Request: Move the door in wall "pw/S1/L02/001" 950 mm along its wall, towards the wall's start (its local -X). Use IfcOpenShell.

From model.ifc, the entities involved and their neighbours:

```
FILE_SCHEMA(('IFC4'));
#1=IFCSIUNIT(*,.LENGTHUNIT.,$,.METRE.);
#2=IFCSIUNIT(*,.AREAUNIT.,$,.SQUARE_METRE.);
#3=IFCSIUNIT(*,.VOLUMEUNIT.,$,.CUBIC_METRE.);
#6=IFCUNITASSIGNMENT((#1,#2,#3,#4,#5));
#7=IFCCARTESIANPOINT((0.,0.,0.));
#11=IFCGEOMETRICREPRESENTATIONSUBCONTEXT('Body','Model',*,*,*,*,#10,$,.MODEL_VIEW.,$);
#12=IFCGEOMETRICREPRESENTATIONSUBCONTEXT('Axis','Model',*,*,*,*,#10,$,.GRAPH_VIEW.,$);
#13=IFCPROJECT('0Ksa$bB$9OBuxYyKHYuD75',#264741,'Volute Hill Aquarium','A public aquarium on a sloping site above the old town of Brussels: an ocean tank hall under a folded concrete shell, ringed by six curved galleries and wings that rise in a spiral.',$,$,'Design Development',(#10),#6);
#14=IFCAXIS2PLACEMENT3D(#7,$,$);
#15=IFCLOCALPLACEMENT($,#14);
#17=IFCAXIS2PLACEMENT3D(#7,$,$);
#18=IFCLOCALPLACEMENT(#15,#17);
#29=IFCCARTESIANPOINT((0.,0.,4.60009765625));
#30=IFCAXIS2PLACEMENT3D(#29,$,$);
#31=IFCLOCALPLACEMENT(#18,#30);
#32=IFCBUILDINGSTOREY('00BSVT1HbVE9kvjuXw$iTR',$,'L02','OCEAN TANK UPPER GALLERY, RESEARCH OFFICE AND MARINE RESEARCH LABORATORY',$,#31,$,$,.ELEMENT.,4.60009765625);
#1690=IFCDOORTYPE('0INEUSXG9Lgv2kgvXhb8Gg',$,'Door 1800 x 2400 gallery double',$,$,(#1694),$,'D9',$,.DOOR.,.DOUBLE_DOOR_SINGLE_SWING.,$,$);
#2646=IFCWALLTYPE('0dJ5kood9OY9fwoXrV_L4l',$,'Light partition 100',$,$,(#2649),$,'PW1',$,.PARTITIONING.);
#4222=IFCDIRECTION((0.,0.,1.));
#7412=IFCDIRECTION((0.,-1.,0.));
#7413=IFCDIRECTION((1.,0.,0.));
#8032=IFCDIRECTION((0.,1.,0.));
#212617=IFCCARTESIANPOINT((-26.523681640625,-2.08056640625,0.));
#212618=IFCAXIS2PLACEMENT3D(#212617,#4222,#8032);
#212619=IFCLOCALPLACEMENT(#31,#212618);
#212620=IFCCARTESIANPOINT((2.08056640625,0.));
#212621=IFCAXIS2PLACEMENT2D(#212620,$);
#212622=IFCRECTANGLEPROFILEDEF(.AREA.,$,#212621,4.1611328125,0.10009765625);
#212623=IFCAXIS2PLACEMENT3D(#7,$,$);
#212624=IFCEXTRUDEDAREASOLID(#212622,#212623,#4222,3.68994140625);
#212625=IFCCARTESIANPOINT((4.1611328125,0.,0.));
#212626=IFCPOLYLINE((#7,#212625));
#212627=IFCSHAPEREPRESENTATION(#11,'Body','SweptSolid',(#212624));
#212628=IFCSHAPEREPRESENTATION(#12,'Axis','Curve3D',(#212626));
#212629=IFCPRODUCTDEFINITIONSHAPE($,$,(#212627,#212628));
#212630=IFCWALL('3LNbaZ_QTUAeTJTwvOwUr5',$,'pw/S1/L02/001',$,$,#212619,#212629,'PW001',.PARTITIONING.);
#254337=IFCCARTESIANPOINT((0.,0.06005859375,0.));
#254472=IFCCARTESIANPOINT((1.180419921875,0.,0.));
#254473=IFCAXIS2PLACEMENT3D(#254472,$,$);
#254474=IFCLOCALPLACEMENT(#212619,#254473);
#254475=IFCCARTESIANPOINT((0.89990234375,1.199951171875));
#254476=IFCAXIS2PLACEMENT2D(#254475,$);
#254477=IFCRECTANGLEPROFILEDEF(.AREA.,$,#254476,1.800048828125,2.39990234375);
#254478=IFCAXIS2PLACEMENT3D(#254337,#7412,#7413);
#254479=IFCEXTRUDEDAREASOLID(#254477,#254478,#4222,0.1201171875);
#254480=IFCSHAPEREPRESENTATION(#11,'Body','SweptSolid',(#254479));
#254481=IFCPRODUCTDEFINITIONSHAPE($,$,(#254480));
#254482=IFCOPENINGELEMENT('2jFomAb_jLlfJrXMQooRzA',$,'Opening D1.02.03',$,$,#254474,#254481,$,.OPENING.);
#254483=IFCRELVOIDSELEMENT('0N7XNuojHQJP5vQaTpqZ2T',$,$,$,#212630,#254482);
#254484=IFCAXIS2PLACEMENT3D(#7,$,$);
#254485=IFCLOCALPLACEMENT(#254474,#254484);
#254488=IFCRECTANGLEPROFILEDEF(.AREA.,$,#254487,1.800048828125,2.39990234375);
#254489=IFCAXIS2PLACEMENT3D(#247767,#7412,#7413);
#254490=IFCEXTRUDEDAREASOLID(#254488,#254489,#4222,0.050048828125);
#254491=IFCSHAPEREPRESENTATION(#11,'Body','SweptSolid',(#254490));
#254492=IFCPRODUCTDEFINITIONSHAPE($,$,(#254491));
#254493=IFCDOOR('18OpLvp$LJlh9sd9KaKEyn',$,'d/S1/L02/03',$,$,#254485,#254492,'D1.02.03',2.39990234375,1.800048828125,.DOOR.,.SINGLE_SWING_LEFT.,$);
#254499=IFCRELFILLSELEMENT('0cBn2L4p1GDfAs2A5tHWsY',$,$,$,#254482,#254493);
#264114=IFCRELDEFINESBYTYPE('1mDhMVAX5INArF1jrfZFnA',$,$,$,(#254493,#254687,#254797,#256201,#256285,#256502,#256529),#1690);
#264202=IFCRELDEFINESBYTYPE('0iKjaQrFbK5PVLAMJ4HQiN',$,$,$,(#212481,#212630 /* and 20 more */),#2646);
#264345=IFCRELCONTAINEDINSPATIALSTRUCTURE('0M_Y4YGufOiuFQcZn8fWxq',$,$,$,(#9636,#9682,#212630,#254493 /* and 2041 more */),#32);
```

```python
import ifcopenshell
import ifcopenshell.api.geometry
import ifcopenshell.util.placement
import ifcopenshell.util.unit

model = ifcopenshell.open("model.ifc")
unit_scale = ifcopenshell.util.unit.calculate_unit_scale(model)

door = model.by_id(254493)
opening = door.FillsVoids[0].RelatingOpeningElement
wall = opening.VoidsElements[0].RelatingBuildingElement

wall_matrix = ifcopenshell.util.placement.get_local_placement(wall.ObjectPlacement)
shift = wall_matrix[:3, 0] * -0.95 / unit_scale
before = ifcopenshell.util.placement.get_local_placement(door.ObjectPlacement)[:3, 3].copy()

# The door is placed relative to its opening, so it follows when the opening moves.
matrix = ifcopenshell.util.placement.get_local_placement(opening.ObjectPlacement)
matrix[:3, 3] += shift
ifcopenshell.api.geometry.edit_object_placement(
    model, product=opening, matrix=matrix, is_si=False, should_transform_children=True
)

after = ifcopenshell.util.placement.get_local_placement(door.ObjectPlacement)[:3, 3]
print("door moved by", (after - before).round(3) + 0.0)

model.write("model-out.ifc")
```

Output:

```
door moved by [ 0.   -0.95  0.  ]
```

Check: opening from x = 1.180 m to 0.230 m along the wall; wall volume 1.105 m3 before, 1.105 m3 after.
